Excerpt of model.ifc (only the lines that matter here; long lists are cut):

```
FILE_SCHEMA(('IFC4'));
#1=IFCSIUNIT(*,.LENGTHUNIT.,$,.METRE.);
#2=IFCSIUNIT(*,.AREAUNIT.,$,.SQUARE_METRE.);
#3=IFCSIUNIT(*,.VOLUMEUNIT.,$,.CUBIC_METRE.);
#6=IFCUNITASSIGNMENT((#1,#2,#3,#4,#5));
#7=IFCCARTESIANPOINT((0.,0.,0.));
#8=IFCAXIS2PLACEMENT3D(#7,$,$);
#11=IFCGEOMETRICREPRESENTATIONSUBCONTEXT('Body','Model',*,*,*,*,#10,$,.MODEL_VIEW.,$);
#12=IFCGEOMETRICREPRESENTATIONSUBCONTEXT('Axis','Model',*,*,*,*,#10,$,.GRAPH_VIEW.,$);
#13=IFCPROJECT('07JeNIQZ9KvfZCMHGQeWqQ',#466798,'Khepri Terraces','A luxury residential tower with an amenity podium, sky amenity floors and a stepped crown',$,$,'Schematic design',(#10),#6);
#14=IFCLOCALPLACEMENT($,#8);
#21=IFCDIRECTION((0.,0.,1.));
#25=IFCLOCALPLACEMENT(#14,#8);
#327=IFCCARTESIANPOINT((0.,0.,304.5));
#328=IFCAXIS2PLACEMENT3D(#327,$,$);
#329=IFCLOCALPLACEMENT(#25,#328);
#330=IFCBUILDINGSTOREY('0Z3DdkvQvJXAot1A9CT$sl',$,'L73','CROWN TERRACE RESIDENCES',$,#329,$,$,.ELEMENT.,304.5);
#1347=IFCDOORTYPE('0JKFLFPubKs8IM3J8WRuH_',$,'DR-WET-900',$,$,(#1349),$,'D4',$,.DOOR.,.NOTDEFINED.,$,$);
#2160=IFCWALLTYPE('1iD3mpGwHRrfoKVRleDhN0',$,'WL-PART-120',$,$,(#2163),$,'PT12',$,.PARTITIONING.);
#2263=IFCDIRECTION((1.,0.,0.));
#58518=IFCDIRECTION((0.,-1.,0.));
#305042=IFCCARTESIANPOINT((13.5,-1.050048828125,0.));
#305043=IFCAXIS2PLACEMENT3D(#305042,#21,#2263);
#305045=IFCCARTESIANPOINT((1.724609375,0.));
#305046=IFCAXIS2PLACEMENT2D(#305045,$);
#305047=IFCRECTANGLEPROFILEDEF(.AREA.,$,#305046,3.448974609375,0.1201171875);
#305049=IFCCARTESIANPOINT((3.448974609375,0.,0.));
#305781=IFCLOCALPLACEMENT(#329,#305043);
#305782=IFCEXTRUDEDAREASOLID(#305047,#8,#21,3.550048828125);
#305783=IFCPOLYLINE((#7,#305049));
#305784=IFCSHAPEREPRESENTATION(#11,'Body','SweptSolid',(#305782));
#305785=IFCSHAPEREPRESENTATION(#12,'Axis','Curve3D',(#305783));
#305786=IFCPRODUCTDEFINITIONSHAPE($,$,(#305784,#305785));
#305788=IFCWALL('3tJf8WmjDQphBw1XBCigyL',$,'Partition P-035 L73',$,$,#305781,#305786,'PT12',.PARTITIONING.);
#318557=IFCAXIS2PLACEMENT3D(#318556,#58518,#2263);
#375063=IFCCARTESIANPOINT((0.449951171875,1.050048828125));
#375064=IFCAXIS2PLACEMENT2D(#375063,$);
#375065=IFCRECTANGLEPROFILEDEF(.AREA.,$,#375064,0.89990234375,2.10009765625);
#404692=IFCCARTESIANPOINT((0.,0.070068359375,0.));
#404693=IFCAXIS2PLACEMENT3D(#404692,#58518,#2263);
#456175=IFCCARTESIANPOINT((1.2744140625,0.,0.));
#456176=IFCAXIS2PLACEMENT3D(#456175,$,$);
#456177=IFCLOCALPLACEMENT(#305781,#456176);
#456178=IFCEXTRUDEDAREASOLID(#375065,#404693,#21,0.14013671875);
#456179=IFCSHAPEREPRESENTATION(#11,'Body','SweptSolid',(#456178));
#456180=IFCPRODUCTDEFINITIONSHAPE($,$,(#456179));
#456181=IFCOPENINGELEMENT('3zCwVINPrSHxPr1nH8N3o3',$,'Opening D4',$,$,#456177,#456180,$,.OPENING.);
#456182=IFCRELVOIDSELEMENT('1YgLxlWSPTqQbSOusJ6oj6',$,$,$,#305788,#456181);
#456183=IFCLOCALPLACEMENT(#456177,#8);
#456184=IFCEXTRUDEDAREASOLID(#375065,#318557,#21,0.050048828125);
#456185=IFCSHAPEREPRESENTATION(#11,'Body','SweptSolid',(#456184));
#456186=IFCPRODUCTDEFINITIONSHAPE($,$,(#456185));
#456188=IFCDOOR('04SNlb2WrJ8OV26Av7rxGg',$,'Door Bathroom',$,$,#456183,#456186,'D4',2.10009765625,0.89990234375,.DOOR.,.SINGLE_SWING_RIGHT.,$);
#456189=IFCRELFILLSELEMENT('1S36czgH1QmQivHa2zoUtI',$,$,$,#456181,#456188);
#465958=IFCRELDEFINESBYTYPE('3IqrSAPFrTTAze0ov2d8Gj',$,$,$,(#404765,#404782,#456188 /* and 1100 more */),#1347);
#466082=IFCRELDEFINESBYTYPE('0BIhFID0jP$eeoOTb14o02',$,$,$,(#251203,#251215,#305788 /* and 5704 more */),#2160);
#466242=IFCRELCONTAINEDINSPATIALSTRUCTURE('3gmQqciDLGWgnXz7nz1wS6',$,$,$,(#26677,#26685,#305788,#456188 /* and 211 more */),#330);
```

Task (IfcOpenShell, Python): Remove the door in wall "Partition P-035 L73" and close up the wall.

```python
import ifcopenshell
import ifcopenshell.api.feature
import ifcopenshell.api.root
import ifcopenshell.geom
import ifcopenshell.util.shape

model = ifcopenshell.open("model.ifc")
settings = ifcopenshell.geom.settings()


def volume(element):
    """Net volume in cubic metres, openings subtracted."""
    shape = ifcopenshell.geom.create_shape(settings, element)
    return ifcopenshell.util.shape.get_volume(shape.geometry)


door = model.by_id(456188)
opening = door.FillsVoids[0].RelatingOpeningElement
wall = opening.VoidsElements[0].RelatingBuildingElement
before = volume(wall)

ifcopenshell.api.root.remove_product(model, product=door)
ifcopenshell.api.feature.remove_feature(model, feature=opening)

after = volume(wall)

print(f"wall volume {before:.3f} -> {after:.3f} m3")

model.write("model-out.ifc")
```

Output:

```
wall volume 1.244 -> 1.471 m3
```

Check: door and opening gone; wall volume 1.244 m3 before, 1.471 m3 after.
